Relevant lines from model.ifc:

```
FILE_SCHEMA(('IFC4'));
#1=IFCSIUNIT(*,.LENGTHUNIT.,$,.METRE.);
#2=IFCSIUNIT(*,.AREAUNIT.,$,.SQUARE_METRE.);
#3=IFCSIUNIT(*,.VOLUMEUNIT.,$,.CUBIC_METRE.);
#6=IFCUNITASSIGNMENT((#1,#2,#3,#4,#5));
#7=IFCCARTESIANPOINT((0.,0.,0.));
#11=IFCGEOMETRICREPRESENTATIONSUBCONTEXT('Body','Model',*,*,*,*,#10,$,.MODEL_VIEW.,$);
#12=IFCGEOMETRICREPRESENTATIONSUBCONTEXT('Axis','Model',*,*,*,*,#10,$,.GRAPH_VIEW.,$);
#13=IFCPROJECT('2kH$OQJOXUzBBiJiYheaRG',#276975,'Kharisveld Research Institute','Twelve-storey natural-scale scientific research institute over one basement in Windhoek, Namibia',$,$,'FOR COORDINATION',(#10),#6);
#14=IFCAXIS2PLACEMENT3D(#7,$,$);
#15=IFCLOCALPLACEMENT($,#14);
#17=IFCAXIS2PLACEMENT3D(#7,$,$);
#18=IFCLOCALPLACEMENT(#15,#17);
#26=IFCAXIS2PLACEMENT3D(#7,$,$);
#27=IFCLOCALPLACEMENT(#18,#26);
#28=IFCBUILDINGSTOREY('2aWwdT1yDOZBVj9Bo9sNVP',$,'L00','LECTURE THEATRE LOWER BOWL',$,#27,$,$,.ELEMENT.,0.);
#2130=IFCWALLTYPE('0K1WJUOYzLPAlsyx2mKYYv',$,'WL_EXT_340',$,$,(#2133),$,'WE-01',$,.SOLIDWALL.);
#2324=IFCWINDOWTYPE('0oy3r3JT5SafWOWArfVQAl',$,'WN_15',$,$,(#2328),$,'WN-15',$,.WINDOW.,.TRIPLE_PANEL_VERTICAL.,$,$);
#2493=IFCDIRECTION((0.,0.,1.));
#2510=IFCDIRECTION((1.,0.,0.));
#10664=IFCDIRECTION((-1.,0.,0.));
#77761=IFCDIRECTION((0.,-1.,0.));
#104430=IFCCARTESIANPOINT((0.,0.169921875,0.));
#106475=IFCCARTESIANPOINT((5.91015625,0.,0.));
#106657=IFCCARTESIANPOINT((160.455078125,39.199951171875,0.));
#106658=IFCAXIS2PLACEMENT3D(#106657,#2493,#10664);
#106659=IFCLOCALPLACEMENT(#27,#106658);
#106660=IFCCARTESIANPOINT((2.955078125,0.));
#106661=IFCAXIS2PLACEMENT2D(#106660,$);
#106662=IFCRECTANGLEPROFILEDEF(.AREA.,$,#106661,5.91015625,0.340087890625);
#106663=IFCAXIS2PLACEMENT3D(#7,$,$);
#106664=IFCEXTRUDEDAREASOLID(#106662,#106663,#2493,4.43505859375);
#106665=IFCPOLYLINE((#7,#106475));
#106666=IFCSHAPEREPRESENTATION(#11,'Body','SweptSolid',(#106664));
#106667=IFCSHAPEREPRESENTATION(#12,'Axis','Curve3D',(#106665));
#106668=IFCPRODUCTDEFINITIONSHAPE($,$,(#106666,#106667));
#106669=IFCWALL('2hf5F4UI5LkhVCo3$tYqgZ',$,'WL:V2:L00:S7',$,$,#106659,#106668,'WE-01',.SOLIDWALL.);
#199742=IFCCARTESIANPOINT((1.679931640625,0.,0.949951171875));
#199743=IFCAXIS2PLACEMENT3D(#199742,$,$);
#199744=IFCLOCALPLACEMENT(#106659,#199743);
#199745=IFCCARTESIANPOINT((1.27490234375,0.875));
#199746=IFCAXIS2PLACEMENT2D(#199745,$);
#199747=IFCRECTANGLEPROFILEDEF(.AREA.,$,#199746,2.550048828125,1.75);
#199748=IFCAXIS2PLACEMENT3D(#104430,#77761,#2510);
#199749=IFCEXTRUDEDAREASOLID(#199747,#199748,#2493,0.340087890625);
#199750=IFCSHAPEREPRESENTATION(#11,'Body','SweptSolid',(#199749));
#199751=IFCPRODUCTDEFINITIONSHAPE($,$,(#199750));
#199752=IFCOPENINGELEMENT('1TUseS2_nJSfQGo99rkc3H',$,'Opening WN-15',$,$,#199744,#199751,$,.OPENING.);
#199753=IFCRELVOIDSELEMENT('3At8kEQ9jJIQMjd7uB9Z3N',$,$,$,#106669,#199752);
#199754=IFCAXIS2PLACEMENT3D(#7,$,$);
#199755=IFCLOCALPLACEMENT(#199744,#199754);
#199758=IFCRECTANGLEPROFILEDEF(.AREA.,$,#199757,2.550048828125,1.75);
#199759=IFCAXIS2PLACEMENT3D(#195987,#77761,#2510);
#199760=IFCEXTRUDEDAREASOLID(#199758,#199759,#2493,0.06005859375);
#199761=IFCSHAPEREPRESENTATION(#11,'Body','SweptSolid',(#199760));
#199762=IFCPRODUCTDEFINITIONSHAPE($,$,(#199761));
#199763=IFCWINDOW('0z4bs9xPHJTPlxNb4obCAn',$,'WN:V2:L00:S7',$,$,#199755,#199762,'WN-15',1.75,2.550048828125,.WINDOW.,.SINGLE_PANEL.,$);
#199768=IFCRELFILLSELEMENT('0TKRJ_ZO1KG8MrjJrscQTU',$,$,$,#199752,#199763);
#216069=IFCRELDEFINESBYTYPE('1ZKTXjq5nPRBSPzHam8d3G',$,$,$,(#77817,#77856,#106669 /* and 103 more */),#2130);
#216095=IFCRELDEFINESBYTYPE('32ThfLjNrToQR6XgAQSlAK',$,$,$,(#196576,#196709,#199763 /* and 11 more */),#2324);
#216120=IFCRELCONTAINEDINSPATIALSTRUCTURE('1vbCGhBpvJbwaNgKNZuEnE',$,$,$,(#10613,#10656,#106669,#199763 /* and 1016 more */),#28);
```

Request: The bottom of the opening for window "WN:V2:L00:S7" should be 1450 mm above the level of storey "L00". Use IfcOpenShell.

```python
import numpy as np
import ifcopenshell
import ifcopenshell.api.geometry
import ifcopenshell.geom
import ifcopenshell.util.element
import ifcopenshell.util.placement
import ifcopenshell.util.shape
import ifcopenshell.util.unit

model = ifcopenshell.open("model.ifc")
unit_scale = ifcopenshell.util.unit.calculate_unit_scale(model)

window = model.by_guid("0z4bs9xPHJTPlxNb4obCAn")
opening = window.FillsVoids[0].RelatingOpeningElement
storey = ifcopenshell.util.element.get_container(window, ifc_class="IfcBuildingStorey")
level = ifcopenshell.util.placement.get_local_placement(storey.ObjectPlacement)[2, 3]

# The opening's origin need not be at the sill, so measure its lowest point.
shape = ifcopenshell.geom.create_shape(ifcopenshell.geom.settings(), opening)
bottom = ifcopenshell.util.shape.get_shape_bottom_elevation(shape, shape.geometry) / unit_scale
dz = level + 1.45 - bottom

shift = np.array([0.0, 0.0, dz])
# The window is placed relative to its opening, so it follows when the opening moves.
matrix = ifcopenshell.util.placement.get_local_placement(opening.ObjectPlacement)
matrix[:3, 3] += shift
ifcopenshell.api.geometry.edit_object_placement(
    model, product=opening, matrix=matrix, is_si=False, should_transform_children=True
)

print(f"moved by {dz * unit_scale:+.3f} m")

model.write("model_edited.ifc")
```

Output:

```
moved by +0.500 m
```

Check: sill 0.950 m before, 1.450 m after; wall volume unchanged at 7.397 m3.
